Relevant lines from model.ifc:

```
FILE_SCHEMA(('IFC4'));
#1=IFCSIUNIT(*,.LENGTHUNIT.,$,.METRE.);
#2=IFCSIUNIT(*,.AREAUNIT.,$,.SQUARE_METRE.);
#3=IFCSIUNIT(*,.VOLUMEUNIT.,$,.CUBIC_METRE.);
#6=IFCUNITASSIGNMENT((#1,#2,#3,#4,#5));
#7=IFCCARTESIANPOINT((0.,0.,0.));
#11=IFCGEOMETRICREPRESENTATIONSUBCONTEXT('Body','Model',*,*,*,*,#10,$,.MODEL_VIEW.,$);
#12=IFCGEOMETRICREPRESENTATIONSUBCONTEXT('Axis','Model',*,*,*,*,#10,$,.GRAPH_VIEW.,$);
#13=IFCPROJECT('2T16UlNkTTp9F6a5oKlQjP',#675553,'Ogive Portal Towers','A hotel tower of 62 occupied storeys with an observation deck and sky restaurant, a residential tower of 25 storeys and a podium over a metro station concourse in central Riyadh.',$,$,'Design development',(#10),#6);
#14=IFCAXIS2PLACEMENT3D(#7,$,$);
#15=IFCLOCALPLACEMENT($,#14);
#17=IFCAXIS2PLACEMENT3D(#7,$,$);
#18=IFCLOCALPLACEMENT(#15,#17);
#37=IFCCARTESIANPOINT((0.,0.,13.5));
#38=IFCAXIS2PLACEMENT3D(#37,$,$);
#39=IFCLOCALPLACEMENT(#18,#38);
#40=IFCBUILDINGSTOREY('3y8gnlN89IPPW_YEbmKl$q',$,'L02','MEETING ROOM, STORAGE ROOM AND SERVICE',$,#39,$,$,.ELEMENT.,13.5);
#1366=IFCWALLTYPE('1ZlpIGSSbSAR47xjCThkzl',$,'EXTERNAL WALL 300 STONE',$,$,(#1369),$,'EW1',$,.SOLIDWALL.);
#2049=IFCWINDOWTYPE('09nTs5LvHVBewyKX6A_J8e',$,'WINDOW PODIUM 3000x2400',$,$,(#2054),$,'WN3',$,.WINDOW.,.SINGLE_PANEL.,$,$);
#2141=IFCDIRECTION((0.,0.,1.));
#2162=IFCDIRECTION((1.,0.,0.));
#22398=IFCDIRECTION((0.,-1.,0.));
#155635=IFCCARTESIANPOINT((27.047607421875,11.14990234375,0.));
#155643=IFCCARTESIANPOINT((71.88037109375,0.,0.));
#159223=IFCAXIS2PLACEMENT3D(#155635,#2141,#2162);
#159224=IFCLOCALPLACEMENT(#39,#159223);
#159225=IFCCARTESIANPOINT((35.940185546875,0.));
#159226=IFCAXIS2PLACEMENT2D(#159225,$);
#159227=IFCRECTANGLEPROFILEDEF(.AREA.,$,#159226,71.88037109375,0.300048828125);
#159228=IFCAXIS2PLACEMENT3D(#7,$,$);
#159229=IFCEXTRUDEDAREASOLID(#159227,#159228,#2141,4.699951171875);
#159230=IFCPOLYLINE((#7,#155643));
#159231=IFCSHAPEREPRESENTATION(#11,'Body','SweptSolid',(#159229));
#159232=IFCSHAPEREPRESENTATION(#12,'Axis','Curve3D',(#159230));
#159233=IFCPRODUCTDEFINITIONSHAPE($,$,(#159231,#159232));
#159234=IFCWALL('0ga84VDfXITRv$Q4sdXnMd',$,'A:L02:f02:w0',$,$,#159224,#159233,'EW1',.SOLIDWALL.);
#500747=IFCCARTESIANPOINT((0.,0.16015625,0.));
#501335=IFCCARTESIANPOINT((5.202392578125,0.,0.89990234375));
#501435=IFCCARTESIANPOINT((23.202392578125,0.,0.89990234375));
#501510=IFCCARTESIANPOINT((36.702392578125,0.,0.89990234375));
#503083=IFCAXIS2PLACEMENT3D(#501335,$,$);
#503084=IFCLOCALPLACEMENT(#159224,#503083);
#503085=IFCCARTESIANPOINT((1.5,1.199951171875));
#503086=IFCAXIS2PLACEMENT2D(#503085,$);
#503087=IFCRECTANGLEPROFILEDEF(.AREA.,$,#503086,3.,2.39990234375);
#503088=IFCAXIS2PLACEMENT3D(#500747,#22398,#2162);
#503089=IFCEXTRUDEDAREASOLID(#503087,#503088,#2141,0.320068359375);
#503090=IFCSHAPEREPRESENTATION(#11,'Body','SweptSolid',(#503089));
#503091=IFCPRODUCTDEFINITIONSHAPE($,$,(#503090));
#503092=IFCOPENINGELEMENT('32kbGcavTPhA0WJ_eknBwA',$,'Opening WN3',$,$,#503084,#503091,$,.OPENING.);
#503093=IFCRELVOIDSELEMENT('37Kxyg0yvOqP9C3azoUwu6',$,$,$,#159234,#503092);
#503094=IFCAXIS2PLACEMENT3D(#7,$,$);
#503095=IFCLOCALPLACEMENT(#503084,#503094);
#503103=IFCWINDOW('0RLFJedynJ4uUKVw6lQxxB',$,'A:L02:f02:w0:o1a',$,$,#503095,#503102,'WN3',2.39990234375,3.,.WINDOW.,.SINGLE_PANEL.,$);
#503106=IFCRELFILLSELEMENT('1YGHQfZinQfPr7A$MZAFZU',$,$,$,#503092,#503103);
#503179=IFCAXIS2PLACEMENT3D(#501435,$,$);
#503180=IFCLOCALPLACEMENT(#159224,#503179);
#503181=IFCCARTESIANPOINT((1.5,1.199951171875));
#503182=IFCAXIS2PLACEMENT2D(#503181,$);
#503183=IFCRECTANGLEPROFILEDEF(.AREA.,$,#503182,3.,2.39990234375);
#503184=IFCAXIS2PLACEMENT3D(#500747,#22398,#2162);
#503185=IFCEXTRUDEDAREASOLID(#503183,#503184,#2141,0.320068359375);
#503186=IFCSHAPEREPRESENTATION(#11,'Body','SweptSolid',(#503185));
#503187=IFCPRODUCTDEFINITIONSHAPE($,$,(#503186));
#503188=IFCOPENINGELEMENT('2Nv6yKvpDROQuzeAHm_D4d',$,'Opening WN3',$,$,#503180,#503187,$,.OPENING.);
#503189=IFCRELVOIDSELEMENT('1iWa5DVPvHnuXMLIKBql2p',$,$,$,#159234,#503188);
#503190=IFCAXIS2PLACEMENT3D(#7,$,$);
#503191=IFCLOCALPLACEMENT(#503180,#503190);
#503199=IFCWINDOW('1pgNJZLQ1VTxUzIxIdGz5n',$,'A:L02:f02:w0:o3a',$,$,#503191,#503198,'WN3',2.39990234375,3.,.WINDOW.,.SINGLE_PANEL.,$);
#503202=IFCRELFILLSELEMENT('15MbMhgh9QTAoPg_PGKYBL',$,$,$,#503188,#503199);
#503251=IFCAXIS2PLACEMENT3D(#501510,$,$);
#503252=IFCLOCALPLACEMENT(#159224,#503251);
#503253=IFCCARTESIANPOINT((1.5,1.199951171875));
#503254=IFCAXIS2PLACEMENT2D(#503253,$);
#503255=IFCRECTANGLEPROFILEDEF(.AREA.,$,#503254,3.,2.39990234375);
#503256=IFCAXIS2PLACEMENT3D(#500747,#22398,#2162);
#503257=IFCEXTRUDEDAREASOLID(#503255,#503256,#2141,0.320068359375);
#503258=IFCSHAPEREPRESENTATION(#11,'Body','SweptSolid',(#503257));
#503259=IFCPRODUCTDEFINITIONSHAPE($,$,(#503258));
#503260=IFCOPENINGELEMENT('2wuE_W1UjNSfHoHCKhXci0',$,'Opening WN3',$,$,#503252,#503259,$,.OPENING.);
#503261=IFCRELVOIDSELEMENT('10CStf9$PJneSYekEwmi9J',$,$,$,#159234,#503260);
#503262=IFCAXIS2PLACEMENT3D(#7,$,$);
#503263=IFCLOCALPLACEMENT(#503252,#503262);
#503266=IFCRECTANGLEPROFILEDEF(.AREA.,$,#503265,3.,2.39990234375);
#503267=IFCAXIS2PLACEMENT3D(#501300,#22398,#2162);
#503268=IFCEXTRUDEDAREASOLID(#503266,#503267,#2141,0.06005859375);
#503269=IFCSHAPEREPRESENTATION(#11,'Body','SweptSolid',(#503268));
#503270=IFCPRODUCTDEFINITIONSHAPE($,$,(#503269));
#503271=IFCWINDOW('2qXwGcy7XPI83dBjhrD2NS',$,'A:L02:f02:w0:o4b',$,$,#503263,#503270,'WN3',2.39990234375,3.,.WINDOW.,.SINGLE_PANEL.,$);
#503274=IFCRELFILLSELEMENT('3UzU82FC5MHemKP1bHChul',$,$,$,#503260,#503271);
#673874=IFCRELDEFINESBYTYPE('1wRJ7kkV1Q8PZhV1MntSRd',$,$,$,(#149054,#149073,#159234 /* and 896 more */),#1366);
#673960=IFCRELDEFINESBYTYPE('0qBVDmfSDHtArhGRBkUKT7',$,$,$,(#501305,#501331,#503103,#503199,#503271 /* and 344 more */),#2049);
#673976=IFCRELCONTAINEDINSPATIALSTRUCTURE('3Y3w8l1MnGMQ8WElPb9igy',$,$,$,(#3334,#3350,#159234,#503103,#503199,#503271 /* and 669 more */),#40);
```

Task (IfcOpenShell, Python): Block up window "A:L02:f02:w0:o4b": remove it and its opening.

```python
import ifcopenshell
import ifcopenshell.api.feature
import ifcopenshell.api.root
import ifcopenshell.geom
import ifcopenshell.util.shape

model = ifcopenshell.open("model.ifc")
settings = ifcopenshell.geom.settings()


def volume(element):
    """Net volume in cubic metres, openings subtracted."""
    shape = ifcopenshell.geom.create_shape(settings, element)
    return ifcopenshell.util.shape.get_volume(shape.geometry)


window = model.by_guid("2qXwGcy7XPI83dBjhrD2NS")
opening = window.FillsVoids[0].RelatingOpeningElement
wall = opening.VoidsElements[0].RelatingBuildingElement
before = volume(wall)

ifcopenshell.api.root.remove_product(model, product=window)
ifcopenshell.api.feature.remove_feature(model, feature=opening)

after = volume(wall)

print(f"wall volume {before:.3f} -> {after:.3f} m3")

model.write("model_updated.ifc")
```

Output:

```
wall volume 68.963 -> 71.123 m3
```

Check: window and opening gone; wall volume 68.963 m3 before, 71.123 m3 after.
